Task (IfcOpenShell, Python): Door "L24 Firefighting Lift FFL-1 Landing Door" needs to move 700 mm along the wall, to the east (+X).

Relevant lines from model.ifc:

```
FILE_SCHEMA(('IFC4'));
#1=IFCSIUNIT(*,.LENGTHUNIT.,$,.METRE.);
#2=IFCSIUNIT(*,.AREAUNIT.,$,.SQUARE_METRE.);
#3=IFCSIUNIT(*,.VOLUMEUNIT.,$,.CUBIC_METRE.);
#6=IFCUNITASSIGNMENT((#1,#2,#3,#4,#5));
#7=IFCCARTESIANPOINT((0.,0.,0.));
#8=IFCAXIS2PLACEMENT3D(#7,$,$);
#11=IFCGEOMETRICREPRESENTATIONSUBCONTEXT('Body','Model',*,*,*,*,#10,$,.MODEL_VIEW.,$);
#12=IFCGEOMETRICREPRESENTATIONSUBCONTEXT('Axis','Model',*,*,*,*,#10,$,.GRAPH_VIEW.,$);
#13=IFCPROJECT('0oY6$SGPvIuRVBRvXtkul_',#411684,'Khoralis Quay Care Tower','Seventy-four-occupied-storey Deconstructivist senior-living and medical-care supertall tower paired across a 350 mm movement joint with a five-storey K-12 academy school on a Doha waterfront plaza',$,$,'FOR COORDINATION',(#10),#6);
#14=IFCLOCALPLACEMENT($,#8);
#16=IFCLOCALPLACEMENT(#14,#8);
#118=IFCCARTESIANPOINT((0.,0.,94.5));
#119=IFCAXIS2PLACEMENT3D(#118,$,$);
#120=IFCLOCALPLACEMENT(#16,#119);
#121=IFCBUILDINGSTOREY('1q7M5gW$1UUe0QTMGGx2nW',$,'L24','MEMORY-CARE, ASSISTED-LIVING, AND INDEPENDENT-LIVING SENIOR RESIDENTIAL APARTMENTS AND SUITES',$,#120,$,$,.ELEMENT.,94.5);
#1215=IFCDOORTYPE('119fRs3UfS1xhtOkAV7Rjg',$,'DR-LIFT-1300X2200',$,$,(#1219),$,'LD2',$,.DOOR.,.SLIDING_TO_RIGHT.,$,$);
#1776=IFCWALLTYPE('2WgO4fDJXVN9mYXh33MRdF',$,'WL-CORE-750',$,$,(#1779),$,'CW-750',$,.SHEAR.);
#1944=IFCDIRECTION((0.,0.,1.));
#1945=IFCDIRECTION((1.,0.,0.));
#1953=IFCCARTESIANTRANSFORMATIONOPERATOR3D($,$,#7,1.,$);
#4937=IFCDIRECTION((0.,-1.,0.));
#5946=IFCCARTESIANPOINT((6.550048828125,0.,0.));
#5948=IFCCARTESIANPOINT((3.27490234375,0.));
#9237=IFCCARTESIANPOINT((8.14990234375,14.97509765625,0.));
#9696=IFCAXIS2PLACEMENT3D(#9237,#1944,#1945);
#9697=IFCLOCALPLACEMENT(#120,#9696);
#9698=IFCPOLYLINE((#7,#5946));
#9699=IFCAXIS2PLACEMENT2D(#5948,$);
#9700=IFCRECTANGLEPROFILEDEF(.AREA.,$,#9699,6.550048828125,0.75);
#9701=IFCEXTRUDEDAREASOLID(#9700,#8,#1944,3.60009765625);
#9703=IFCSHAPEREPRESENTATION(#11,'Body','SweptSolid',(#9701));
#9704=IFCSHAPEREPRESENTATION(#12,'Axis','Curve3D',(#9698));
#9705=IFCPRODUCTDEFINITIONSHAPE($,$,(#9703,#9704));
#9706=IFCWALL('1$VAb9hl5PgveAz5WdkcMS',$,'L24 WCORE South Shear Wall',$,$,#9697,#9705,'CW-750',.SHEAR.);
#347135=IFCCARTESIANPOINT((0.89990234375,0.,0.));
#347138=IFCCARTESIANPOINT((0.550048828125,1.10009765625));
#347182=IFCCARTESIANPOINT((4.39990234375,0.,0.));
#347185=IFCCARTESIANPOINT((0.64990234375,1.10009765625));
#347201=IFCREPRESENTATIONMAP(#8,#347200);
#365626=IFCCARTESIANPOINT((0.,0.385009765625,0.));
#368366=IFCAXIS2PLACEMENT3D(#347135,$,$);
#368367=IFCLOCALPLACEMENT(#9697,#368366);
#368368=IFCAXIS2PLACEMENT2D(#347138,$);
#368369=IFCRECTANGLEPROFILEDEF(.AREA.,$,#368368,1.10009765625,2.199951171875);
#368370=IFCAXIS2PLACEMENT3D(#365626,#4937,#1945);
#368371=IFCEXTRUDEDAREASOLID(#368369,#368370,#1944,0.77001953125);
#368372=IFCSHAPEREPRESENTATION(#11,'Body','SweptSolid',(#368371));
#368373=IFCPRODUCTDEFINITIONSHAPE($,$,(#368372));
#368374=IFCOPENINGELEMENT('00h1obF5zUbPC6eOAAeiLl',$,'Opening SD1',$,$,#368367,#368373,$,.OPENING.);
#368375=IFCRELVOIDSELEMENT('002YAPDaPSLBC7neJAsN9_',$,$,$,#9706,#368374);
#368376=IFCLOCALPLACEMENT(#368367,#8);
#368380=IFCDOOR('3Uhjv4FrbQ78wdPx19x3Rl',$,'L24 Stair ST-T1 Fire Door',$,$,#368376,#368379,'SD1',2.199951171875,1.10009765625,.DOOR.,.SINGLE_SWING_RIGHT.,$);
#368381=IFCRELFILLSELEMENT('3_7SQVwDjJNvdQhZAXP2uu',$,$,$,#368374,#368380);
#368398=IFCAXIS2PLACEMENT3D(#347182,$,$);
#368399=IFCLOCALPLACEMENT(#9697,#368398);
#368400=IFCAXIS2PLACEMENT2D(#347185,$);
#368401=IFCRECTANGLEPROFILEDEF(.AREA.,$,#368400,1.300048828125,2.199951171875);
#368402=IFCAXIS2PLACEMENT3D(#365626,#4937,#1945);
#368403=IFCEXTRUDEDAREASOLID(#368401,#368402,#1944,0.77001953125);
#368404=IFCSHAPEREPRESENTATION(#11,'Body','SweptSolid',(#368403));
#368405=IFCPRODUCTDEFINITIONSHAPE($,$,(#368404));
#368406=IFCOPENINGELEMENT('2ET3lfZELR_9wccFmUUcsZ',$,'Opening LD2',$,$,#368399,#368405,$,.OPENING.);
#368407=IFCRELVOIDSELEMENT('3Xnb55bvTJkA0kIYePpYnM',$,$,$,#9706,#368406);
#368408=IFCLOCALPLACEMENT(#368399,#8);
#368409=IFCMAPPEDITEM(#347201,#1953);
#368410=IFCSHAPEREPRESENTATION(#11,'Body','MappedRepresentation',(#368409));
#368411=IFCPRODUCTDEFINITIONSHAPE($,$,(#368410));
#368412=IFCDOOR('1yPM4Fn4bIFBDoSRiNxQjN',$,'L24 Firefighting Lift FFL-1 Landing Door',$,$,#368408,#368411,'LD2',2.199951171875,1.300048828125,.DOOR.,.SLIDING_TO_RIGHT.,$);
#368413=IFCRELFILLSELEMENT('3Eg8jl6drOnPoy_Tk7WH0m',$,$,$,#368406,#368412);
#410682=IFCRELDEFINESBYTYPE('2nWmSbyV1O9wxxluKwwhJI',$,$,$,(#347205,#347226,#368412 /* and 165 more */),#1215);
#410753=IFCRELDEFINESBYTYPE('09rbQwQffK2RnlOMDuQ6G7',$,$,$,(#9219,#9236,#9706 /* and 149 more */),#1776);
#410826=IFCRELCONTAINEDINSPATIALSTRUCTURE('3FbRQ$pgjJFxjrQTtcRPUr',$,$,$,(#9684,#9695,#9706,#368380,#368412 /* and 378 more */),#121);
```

```python
import ifcopenshell
import ifcopenshell.api.geometry
import ifcopenshell.util.placement
import ifcopenshell.util.unit

model = ifcopenshell.open("model.ifc")
unit_scale = ifcopenshell.util.unit.calculate_unit_scale(model)

door = model.by_id(368412)
opening = door.FillsVoids[0].RelatingOpeningElement
wall = opening.VoidsElements[0].RelatingBuildingElement

wall_matrix = ifcopenshell.util.placement.get_local_placement(wall.ObjectPlacement)
shift = wall_matrix[:3, 0] * 0.7 / unit_scale
before = ifcopenshell.util.placement.get_local_placement(door.ObjectPlacement)[:3, 3].copy()

# The door is placed relative to its opening, so it follows when the opening moves.
matrix = ifcopenshell.util.placement.get_local_placement(opening.ObjectPlacement)
matrix[:3, 3] += shift
ifcopenshell.api.geometry.edit_object_placement(
    model, product=opening, matrix=matrix, is_si=False, should_transform_children=True
)

after = ifcopenshell.util.placement.get_local_placement(door.ObjectPlacement)[:3, 3]
print("door moved by", (after - before).round(3) + 0.0)

model.write("model_edited.ifc")
```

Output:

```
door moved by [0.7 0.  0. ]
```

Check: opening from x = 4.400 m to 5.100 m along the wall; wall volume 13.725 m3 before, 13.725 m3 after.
